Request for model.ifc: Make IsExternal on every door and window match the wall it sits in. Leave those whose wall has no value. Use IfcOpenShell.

First a look at what the model holds.

```python
import ifcopenshell
import ifcopenshell.util.element

model = ifcopenshell.open("model.ifc")
print(model.schema)
seen = {}
for e in model.by_type("IfcDoor") + model.by_type("IfcWindow"):
    if not e.FillsVoids:
        continue
    host = e.FillsVoids[0].RelatingOpeningElement.VoidsElements[0].RelatingBuildingElement
    own = ifcopenshell.util.element.get_pset(e, f"Pset_{e.is_a()[3:].removesuffix('StandardCase')}Common", "IsExternal")
    wall = ifcopenshell.util.element.get_pset(host, "Pset_WallCommon", "IsExternal")
    seen[e.is_a(), own, wall] = seen.get((e.is_a(), own, wall), 0) + 1
for (cls, own, wall), count in sorted(seen.items(), key=str):
    print(count, cls, "IsExternal:", own, "| host wall:", wall)
```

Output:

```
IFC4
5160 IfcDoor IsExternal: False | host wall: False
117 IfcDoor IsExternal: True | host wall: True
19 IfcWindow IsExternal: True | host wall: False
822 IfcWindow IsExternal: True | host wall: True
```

```python
import ifcopenshell
import ifcopenshell.api.pset
import ifcopenshell.util.element

model = ifcopenshell.open("model.ifc")

count = 0
for ifc_class, pset_name in (("IfcDoor", "Pset_DoorCommon"), ("IfcWindow", "Pset_WindowCommon")):
    for e in model.by_type(ifc_class):
        if not e.FillsVoids:
            continue
        host = e.FillsVoids[0].RelatingOpeningElement.VoidsElements[0].RelatingBuildingElement
        external = ifcopenshell.util.element.get_pset(host, "Pset_WallCommon", "IsExternal")
        if external is None or ifcopenshell.util.element.get_pset(e, pset_name, "IsExternal") == external:
            continue
        pset = ifcopenshell.api.pset.add_pset(model, product=e, name=pset_name)
        ifcopenshell.api.pset.edit_pset(model, pset=pset, properties={"IsExternal": external})
        count += 1

print(count, "updated")

model.write("model_rev.ifc")
```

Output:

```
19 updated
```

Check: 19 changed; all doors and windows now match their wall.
